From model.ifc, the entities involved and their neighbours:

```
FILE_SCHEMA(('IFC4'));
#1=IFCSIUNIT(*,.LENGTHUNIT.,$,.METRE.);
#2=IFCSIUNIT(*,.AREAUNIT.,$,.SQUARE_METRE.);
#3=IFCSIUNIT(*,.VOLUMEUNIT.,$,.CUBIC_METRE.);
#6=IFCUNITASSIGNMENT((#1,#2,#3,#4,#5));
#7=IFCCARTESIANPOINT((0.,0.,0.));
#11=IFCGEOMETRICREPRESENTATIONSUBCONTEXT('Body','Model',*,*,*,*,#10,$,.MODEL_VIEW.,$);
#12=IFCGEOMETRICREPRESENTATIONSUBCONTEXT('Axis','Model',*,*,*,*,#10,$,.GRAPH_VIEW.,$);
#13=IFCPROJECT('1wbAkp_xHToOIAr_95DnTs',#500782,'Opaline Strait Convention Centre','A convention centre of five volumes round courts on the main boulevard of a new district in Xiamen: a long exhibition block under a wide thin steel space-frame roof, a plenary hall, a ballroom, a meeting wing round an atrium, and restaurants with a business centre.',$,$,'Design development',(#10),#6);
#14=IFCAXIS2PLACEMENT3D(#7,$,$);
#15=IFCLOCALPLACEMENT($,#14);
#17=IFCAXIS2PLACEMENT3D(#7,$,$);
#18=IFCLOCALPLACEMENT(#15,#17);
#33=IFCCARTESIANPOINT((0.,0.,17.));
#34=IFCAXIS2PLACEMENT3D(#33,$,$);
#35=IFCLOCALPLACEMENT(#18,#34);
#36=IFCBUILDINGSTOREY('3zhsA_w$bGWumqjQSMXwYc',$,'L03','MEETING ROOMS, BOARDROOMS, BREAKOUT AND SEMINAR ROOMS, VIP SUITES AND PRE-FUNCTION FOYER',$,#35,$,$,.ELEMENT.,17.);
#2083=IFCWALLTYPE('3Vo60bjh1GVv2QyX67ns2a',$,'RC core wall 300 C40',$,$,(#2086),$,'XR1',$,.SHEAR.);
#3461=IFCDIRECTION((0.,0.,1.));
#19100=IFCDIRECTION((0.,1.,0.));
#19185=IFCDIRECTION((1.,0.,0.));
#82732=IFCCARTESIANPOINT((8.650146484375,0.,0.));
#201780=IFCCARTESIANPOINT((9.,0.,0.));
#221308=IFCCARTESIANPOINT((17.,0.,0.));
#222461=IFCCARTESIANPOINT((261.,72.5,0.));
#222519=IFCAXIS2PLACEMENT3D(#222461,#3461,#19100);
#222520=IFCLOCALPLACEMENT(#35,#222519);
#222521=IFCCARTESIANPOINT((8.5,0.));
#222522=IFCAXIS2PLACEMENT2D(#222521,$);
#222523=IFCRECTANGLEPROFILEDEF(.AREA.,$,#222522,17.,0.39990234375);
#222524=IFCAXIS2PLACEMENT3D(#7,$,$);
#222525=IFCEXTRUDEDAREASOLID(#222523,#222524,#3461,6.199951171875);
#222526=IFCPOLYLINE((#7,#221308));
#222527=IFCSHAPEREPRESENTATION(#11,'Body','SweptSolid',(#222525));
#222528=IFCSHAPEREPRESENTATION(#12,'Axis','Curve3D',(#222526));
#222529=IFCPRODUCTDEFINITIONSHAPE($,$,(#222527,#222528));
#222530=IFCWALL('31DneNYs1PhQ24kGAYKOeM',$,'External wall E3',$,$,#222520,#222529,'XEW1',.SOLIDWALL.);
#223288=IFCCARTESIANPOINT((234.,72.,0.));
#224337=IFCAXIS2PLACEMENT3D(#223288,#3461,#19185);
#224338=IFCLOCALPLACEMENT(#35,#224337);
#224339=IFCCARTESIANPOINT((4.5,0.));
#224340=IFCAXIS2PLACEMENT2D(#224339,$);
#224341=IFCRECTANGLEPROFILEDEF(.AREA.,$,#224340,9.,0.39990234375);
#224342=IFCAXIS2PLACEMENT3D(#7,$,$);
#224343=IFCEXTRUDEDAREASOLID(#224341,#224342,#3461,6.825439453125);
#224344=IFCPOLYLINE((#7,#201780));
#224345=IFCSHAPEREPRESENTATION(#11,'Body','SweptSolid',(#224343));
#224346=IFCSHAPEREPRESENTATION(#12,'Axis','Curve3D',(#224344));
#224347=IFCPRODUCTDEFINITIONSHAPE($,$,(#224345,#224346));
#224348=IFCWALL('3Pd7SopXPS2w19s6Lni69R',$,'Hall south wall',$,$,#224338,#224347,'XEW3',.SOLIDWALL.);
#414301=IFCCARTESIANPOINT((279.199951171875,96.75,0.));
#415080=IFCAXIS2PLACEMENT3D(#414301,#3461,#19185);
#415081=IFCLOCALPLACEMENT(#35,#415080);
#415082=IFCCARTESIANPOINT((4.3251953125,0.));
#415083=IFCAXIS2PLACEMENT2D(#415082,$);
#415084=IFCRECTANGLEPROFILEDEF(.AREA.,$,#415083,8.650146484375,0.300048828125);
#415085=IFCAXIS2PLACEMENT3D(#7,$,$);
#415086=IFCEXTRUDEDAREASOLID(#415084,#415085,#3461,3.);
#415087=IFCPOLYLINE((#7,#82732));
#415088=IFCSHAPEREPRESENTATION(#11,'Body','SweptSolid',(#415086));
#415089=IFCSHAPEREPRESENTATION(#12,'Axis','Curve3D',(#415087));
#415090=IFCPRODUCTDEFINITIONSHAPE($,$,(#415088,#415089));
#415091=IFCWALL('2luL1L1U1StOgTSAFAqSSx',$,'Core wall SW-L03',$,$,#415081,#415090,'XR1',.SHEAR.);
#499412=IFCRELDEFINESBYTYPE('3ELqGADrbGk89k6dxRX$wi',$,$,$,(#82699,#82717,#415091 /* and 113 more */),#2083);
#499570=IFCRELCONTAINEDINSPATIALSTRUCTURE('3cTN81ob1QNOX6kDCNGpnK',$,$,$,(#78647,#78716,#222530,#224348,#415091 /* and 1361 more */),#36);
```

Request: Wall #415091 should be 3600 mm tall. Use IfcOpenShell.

```python
import ifcopenshell
import ifcopenshell.geom
import ifcopenshell.util.representation
import ifcopenshell.util.shape
import ifcopenshell.util.unit

model = ifcopenshell.open("model.ifc")
unit_scale = ifcopenshell.util.unit.calculate_unit_scale(model)
settings = ifcopenshell.geom.settings()


def volume(element):
    """Net volume in cubic metres, openings subtracted."""
    shape = ifcopenshell.geom.create_shape(settings, element)
    return ifcopenshell.util.shape.get_volume(shape.geometry)


wall = model.by_guid("2luL1L1U1StOgTSAFAqSSx")
before = volume(wall)

body = ifcopenshell.util.representation.get_representation(wall, "Model", "Body")
solid = body.Items[0]
old_height = solid.Depth
solid.Depth = 3.6 / unit_scale
after = volume(wall)

print(f"height {old_height:g} -> {solid.Depth:g}, volume {before:.3f} -> {after:.3f} m3")

model.write("model_v2.ifc")
```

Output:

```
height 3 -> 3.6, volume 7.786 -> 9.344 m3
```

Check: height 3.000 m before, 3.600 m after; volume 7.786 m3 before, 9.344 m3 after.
